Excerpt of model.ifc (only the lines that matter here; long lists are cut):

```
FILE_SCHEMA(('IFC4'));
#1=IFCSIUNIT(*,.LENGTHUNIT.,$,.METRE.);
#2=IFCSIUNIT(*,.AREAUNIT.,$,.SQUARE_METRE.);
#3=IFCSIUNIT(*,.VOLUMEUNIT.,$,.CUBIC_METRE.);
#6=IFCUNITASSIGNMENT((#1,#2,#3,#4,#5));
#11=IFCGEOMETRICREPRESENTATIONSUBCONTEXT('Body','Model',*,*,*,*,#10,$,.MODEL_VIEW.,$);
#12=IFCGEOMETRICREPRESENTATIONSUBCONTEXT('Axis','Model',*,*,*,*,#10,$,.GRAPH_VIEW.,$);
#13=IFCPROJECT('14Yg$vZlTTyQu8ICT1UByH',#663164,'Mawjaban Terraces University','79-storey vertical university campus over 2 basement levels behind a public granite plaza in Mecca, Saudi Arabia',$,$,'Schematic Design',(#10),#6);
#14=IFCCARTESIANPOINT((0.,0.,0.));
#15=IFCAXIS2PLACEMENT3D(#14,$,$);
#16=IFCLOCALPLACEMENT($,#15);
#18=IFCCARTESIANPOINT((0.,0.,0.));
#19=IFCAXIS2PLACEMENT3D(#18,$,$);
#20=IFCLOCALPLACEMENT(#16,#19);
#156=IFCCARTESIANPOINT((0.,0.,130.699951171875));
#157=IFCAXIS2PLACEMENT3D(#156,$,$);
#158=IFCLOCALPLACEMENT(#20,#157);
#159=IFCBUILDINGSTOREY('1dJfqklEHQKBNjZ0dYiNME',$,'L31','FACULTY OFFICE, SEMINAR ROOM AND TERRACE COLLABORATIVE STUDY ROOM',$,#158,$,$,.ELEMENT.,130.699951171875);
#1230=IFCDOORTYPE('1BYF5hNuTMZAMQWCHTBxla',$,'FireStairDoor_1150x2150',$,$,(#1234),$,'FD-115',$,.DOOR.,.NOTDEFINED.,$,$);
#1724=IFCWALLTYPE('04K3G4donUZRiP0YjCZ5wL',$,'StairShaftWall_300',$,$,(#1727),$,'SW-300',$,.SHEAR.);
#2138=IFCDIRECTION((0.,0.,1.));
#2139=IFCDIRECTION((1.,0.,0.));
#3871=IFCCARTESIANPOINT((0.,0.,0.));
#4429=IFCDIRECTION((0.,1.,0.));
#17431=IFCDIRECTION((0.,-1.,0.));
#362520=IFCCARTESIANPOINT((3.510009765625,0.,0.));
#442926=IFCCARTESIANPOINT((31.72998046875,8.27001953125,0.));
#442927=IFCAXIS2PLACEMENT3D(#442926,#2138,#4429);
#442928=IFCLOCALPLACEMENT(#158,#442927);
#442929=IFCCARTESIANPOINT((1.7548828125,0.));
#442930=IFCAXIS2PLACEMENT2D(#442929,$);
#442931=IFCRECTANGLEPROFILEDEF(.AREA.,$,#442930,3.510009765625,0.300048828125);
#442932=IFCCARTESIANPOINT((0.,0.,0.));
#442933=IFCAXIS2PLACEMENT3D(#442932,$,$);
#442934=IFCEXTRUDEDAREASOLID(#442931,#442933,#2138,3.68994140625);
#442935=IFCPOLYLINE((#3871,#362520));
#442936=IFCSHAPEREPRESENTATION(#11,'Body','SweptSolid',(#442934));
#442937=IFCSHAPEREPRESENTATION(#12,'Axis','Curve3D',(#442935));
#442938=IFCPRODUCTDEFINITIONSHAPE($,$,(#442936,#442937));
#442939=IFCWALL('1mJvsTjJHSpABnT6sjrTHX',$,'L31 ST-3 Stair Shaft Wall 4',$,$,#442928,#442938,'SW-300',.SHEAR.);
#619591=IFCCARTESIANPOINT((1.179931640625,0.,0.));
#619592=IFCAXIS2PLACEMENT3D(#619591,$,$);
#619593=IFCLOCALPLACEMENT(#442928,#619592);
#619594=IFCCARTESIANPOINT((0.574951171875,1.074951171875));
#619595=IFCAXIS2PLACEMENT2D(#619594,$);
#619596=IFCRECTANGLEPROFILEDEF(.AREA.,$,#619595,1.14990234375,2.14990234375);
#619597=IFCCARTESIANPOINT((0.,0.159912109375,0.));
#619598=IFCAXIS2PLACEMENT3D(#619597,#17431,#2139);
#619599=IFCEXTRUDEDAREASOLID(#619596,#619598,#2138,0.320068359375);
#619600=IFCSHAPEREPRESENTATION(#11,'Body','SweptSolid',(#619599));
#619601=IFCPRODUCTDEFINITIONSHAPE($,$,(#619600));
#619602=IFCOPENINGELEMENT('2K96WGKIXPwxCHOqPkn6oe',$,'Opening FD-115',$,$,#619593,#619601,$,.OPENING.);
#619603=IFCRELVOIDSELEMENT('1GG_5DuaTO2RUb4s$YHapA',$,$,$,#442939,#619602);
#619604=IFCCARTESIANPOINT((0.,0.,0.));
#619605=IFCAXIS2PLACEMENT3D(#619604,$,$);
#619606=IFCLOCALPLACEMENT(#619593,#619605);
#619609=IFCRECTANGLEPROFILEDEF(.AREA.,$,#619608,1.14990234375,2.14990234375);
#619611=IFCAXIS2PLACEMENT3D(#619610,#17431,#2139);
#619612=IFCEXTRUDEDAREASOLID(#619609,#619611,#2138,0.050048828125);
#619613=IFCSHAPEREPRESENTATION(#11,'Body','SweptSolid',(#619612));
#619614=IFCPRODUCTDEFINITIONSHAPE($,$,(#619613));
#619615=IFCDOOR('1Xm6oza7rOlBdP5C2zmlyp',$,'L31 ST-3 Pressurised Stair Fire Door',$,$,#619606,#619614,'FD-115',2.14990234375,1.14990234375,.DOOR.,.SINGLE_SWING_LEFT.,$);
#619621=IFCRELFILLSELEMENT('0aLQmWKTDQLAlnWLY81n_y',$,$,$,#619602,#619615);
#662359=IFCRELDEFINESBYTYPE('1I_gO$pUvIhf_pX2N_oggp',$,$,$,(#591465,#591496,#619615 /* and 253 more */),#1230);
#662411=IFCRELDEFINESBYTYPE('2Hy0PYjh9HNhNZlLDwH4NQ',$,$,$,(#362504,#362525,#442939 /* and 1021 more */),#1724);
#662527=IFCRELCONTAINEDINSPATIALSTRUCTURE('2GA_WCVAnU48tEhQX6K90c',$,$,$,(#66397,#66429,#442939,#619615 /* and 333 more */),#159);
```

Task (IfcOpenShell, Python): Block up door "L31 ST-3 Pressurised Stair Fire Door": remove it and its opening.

```python
import ifcopenshell
import ifcopenshell.api.feature
import ifcopenshell.api.root
import ifcopenshell.geom
import ifcopenshell.util.shape

model = ifcopenshell.open("model.ifc")
settings = ifcopenshell.geom.settings()


def volume(element):
    """Net volume in cubic metres, openings subtracted."""
    shape = ifcopenshell.geom.create_shape(settings, element)
    return ifcopenshell.util.shape.get_volume(shape.geometry)


door = model.by_guid("1Xm6oza7rOlBdP5C2zmlyp")
opening = door.FillsVoids[0].RelatingOpeningElement
wall = opening.VoidsElements[0].RelatingBuildingElement
before = volume(wall)

ifcopenshell.api.root.remove_product(model, product=door)
ifcopenshell.api.feature.remove_feature(model, feature=opening)

after = volume(wall)

print(f"wall volume {before:.3f} -> {after:.3f} m3")

model.write("model_updated.ifc")
```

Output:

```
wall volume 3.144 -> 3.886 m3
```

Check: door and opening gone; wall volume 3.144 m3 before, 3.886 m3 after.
